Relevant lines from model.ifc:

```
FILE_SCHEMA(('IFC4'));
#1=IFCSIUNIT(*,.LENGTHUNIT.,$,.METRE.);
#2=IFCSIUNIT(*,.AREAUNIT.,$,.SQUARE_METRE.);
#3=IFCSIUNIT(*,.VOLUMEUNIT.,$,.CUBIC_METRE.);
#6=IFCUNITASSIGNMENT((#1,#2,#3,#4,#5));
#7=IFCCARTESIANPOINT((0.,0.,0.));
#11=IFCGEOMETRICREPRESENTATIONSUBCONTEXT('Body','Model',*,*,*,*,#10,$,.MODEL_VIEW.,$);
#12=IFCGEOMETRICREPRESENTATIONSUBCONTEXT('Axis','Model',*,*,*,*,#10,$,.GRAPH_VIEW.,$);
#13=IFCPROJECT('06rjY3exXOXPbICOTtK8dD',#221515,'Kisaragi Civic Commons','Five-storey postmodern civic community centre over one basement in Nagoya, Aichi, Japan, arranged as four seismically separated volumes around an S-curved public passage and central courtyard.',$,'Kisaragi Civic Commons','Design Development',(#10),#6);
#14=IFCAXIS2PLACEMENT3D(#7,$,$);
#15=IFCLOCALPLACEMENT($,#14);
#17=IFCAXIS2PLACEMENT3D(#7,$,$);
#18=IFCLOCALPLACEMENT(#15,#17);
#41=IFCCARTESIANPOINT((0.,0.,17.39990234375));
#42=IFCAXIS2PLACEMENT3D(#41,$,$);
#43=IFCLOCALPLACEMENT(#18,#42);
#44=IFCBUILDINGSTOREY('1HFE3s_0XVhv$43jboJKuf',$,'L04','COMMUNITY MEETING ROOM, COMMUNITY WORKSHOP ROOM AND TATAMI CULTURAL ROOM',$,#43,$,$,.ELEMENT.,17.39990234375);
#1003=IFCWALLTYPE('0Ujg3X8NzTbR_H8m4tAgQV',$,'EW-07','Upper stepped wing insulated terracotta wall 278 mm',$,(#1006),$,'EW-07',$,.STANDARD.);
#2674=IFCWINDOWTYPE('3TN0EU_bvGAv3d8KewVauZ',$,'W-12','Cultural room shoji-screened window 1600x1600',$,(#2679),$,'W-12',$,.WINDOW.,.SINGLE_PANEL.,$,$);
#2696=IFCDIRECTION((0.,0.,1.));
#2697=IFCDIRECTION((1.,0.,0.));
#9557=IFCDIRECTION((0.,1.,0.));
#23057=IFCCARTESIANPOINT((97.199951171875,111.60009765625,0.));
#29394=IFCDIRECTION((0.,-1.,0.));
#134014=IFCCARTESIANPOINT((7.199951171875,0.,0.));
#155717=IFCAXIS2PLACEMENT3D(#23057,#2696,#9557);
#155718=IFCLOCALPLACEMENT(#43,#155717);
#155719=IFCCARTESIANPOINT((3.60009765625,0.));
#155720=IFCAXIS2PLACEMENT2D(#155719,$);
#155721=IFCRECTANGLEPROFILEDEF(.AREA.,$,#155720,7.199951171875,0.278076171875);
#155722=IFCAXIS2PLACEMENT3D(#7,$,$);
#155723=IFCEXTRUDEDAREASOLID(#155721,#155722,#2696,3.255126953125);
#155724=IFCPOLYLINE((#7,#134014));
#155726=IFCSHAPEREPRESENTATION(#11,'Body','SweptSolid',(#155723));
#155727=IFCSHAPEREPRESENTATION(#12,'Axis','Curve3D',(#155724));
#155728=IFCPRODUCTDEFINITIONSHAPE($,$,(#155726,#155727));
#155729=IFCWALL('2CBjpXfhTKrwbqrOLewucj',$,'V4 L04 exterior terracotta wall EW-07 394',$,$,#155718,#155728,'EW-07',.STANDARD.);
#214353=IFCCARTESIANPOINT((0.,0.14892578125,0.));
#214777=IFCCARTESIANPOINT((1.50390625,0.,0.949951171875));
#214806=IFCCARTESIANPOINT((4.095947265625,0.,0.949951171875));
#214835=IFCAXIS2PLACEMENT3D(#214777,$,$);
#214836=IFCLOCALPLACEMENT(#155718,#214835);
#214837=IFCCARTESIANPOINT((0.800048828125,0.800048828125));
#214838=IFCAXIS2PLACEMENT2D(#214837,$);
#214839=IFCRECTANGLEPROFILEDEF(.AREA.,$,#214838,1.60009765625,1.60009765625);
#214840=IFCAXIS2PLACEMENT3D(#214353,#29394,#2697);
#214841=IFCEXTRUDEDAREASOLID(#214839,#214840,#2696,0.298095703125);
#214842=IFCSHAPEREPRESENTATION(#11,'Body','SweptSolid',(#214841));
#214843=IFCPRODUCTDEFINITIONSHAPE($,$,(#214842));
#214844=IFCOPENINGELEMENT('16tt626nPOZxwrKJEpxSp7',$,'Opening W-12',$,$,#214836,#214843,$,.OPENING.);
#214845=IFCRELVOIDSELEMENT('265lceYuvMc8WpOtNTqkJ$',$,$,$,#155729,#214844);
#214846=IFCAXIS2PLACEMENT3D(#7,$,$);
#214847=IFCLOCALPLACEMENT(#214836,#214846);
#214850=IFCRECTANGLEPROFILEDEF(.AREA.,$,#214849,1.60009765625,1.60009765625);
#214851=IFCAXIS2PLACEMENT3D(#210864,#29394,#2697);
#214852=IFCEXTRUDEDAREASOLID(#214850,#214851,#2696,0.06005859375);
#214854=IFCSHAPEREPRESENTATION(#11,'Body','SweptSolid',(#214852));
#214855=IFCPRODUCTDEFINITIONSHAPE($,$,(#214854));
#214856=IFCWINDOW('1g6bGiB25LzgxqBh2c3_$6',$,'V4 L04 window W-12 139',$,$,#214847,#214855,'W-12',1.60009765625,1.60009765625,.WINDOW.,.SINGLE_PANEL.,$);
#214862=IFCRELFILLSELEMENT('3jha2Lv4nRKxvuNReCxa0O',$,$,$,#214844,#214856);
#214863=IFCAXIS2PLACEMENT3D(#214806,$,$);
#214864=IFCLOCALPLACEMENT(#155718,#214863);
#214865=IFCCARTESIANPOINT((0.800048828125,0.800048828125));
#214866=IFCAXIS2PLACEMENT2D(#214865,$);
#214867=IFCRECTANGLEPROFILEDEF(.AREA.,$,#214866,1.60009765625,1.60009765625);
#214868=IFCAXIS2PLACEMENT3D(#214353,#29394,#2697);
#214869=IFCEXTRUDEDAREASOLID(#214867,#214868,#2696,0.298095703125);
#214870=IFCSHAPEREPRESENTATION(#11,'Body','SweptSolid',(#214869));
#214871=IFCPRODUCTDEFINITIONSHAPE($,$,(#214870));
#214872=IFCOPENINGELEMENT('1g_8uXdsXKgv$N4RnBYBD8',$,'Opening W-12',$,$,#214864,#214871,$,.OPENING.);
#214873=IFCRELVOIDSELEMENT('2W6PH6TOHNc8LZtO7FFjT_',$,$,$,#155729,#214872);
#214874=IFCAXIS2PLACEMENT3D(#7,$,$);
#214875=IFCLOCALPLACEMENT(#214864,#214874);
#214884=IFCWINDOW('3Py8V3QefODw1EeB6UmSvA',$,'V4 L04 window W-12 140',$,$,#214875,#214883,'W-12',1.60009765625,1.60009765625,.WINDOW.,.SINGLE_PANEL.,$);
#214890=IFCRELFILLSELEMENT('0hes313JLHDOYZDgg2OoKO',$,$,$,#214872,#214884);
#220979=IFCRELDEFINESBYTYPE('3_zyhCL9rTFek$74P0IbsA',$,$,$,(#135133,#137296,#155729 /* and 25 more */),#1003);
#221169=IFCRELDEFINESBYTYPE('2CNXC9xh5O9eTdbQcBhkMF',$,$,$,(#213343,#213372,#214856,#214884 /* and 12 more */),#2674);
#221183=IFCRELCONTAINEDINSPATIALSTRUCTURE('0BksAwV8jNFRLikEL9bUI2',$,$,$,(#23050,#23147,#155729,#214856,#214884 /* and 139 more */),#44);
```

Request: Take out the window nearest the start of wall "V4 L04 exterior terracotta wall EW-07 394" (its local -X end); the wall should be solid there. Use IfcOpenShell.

```python
import ifcopenshell
import ifcopenshell.api.feature
import ifcopenshell.api.root
import ifcopenshell.geom
import ifcopenshell.util.shape

model = ifcopenshell.open("model.ifc")
settings = ifcopenshell.geom.settings()


def volume(element):
    """Net volume in cubic metres, openings subtracted."""
    shape = ifcopenshell.geom.create_shape(settings, element)
    return ifcopenshell.util.shape.get_volume(shape.geometry)


window = model.by_id(214856)
opening = window.FillsVoids[0].RelatingOpeningElement
wall = opening.VoidsElements[0].RelatingBuildingElement
before = volume(wall)

ifcopenshell.api.root.remove_product(model, product=window)
ifcopenshell.api.feature.remove_feature(model, feature=opening)

after = volume(wall)

print(f"wall volume {before:.3f} -> {after:.3f} m3")

model.write("model_updated.ifc")
```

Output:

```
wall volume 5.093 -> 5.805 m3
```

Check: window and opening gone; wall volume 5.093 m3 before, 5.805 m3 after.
